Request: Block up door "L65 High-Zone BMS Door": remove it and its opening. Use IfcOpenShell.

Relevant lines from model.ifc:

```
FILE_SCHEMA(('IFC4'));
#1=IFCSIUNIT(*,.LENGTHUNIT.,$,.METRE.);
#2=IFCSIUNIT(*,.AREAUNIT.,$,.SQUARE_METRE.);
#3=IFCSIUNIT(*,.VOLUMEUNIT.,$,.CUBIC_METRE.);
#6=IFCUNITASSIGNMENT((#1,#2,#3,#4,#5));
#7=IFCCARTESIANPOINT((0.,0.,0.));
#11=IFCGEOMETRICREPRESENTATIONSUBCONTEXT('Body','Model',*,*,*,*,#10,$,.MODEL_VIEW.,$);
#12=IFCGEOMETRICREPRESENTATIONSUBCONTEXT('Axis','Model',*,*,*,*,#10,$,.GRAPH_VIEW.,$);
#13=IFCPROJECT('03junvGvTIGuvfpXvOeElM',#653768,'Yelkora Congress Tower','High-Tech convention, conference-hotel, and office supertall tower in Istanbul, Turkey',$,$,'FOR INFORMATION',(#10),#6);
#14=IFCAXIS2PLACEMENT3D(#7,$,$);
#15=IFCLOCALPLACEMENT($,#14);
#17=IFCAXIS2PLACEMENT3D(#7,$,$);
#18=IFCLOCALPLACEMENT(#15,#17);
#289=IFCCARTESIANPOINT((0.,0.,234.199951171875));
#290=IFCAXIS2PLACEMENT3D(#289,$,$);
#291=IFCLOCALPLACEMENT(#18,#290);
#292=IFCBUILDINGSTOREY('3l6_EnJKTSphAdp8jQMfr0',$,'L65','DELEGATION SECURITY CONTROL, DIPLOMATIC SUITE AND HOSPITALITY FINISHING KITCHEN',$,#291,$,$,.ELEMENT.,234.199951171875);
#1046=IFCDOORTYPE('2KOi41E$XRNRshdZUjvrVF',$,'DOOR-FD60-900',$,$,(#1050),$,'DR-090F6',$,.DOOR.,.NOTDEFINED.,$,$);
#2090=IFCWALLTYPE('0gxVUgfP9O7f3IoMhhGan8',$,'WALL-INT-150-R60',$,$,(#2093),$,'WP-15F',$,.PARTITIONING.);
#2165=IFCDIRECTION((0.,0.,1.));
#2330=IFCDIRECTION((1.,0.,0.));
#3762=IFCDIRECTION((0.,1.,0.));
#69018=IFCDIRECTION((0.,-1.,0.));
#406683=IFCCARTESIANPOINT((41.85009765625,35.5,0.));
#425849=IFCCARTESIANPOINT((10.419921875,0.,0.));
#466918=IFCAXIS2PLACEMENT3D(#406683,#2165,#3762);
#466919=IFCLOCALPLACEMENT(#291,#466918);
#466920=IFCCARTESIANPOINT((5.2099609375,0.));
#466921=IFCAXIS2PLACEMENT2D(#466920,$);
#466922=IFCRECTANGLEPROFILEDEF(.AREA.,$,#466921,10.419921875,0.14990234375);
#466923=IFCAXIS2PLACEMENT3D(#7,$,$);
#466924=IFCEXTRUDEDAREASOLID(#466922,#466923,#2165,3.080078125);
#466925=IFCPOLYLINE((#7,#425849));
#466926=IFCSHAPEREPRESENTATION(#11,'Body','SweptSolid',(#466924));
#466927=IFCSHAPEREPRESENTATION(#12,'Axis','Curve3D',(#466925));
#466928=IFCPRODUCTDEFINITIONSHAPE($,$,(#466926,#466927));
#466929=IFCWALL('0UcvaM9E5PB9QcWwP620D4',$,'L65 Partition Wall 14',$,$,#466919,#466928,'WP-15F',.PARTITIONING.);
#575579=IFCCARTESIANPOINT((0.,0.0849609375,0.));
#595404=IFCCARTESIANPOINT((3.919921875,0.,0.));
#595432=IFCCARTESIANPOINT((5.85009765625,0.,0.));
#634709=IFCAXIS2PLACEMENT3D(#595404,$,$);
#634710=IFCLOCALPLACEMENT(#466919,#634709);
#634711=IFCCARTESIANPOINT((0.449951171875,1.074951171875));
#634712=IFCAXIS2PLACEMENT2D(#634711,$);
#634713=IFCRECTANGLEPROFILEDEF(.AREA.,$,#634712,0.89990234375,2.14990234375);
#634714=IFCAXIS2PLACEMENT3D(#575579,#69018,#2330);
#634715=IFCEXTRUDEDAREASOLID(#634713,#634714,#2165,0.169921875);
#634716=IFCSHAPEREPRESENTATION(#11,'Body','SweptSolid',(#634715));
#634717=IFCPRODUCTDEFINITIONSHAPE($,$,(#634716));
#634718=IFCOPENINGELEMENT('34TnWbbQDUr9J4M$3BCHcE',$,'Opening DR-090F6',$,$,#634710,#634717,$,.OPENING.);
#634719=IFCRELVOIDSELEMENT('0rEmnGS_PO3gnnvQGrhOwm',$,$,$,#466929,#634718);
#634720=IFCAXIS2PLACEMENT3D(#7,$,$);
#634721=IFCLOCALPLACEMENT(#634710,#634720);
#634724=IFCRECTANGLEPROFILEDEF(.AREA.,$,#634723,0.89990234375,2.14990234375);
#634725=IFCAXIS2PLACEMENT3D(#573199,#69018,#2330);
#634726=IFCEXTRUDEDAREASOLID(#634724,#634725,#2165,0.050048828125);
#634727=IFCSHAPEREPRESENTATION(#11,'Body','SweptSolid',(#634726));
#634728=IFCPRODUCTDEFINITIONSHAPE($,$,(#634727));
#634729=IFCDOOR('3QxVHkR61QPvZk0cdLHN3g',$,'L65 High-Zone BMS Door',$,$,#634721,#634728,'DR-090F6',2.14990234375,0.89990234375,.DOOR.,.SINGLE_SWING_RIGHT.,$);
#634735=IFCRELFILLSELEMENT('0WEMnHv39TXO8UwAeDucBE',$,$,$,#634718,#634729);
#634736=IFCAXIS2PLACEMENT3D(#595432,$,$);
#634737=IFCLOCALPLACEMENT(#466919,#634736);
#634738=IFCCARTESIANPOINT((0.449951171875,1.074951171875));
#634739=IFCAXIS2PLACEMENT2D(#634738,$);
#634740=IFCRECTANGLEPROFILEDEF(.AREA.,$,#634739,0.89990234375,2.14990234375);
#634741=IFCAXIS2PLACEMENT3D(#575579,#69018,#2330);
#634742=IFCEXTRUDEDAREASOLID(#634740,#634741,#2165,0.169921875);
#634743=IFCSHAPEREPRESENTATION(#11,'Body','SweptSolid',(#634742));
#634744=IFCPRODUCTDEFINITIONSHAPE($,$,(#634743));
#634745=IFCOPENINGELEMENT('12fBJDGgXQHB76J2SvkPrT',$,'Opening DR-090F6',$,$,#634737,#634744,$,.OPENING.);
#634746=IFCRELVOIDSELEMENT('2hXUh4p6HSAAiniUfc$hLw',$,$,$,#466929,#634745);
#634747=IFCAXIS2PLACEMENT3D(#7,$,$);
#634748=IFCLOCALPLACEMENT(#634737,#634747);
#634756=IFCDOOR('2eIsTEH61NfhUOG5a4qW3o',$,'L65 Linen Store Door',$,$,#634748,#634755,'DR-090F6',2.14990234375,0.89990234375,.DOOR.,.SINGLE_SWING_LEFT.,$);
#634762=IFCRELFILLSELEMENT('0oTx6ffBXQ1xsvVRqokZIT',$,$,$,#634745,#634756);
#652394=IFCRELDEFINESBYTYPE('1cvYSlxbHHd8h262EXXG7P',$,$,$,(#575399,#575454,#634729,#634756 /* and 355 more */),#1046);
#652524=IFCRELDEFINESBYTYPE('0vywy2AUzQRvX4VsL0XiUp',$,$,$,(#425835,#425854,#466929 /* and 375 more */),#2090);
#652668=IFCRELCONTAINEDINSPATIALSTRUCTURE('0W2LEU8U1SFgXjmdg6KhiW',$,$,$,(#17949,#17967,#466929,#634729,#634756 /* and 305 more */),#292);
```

```python
import ifcopenshell
import ifcopenshell.api.feature
import ifcopenshell.api.root
import ifcopenshell.geom
import ifcopenshell.util.shape

model = ifcopenshell.open("model.ifc")
settings = ifcopenshell.geom.settings()


def volume(element):
    """Net volume in cubic metres, openings subtracted."""
    shape = ifcopenshell.geom.create_shape(settings, element)
    return ifcopenshell.util.shape.get_volume(shape.geometry)


door = model.by_guid("3QxVHkR61QPvZk0cdLHN3g")
opening = door.FillsVoids[0].RelatingOpeningElement
wall = opening.VoidsElements[0].RelatingBuildingElement
before = volume(wall)

ifcopenshell.api.root.remove_product(model, product=door)
ifcopenshell.api.feature.remove_feature(model, feature=opening)

after = volume(wall)

print(f"wall volume {before:.3f} -> {after:.3f} m3")

model.write("model-out.ifc")
```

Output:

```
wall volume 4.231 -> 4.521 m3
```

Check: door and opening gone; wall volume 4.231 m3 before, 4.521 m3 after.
